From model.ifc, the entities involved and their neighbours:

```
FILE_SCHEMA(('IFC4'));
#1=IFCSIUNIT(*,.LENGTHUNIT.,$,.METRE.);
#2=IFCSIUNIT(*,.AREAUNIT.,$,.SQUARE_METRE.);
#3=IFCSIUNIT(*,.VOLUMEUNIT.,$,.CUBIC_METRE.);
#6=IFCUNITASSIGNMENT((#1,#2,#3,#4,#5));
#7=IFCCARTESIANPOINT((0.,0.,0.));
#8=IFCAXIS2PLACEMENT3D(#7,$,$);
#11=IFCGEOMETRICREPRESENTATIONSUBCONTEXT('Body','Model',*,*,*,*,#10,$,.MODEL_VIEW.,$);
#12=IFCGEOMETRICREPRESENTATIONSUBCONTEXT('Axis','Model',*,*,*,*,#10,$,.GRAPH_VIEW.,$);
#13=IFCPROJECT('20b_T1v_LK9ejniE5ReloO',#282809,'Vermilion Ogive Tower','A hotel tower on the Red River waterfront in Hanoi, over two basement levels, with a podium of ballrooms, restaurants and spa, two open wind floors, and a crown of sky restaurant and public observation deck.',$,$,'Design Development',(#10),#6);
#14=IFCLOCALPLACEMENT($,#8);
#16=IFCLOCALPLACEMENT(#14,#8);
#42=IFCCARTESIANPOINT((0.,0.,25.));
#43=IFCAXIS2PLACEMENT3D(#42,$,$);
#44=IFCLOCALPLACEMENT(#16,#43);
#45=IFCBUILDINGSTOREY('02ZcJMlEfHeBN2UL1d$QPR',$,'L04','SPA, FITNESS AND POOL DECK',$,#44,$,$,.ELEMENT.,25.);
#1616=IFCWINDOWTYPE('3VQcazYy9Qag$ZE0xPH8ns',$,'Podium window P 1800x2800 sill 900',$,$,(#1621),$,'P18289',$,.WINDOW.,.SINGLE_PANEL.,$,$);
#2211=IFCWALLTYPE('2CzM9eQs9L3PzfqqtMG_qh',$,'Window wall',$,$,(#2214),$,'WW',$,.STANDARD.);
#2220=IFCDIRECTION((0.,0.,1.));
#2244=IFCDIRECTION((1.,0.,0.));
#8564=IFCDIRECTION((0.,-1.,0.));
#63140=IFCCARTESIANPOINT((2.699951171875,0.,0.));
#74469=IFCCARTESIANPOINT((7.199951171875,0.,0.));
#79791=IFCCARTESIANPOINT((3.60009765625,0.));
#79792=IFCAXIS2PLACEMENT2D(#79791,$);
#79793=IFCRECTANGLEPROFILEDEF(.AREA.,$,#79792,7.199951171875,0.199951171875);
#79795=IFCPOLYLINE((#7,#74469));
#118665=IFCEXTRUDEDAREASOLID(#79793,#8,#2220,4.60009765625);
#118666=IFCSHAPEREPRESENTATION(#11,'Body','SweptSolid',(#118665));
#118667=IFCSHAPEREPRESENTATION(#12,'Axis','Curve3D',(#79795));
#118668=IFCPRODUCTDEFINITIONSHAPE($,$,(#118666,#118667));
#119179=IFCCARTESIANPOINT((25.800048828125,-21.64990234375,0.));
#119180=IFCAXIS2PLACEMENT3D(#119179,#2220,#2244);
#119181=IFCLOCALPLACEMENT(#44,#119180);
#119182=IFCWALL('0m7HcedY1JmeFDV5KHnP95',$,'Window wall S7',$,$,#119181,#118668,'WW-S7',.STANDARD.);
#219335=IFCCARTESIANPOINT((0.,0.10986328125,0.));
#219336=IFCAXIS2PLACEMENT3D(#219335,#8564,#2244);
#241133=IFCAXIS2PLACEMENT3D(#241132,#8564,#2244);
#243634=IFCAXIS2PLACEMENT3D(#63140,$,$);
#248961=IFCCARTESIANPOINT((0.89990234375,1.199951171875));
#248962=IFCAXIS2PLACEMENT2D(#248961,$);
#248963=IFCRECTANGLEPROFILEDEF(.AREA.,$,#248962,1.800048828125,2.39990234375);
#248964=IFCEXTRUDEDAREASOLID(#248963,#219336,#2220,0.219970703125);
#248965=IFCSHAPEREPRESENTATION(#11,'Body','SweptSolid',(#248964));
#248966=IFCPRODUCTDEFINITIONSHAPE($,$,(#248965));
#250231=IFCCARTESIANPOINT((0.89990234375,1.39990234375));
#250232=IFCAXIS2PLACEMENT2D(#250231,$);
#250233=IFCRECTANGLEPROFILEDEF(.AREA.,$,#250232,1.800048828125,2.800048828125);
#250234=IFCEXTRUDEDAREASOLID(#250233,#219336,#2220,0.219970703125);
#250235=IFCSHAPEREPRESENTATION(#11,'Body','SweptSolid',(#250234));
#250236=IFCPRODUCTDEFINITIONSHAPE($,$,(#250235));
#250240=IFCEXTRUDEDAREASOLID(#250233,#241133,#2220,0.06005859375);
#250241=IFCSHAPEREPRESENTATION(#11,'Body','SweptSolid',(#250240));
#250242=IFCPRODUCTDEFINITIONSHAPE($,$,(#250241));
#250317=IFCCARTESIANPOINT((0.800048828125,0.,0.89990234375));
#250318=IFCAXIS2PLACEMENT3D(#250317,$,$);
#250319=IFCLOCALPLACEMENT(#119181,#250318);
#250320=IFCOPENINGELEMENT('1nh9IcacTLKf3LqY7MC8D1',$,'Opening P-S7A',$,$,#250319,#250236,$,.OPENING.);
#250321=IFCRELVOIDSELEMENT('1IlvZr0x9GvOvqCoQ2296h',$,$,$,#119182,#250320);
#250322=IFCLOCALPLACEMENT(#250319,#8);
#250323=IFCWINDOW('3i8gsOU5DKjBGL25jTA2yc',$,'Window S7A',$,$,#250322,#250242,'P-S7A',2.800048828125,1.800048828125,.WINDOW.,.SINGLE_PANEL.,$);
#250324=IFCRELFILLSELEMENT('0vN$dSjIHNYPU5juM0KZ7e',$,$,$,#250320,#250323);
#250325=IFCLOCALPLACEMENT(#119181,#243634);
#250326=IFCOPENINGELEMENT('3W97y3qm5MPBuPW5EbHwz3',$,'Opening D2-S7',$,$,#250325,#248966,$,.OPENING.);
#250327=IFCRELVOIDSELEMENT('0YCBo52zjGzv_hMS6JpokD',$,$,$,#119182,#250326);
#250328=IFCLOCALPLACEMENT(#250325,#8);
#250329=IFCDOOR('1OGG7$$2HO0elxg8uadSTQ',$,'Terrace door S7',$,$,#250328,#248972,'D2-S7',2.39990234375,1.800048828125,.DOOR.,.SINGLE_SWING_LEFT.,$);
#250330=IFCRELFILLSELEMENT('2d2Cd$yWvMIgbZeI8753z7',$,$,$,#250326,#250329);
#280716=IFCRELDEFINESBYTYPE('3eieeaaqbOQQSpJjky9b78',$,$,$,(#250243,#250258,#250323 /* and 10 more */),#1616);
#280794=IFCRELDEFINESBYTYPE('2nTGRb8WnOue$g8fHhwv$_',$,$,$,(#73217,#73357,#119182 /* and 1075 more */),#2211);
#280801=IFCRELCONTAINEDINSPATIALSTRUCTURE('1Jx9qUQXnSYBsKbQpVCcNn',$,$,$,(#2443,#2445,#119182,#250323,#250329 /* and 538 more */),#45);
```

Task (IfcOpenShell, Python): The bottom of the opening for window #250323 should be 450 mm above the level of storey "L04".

```python
import numpy as np
import ifcopenshell
import ifcopenshell.api.geometry
import ifcopenshell.geom
import ifcopenshell.util.element
import ifcopenshell.util.placement
import ifcopenshell.util.shape
import ifcopenshell.util.unit

model = ifcopenshell.open("model.ifc")
unit_scale = ifcopenshell.util.unit.calculate_unit_scale(model)

window = model.by_guid("3i8gsOU5DKjBGL25jTA2yc")
opening = window.FillsVoids[0].RelatingOpeningElement
storey = ifcopenshell.util.element.get_container(window, ifc_class="IfcBuildingStorey")
level = ifcopenshell.util.placement.get_local_placement(storey.ObjectPlacement)[2, 3]

# The opening's origin need not be at the sill, so measure its lowest point.
shape = ifcopenshell.geom.create_shape(ifcopenshell.geom.settings(), opening)
bottom = ifcopenshell.util.shape.get_shape_bottom_elevation(shape, shape.geometry) / unit_scale
dz = level + 0.45 - bottom

shift = np.array([0.0, 0.0, dz])
# The window is placed relative to its opening, so it follows when the opening moves.
matrix = ifcopenshell.util.placement.get_local_placement(opening.ObjectPlacement)
matrix[:3, 3] += shift
ifcopenshell.api.geometry.edit_object_placement(
    model, product=opening, matrix=matrix, is_si=False, should_transform_children=True
)

print(f"moved by {dz * unit_scale:+.3f} m")

model.write("model_edited.ifc")
```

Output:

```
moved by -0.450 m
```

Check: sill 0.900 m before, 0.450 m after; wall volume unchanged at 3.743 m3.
